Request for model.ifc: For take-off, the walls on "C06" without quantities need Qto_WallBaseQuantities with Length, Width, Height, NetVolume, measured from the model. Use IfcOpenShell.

First a look at what the model holds.

```python
import ifcopenshell
import ifcopenshell.util.element
import ifcopenshell.util.unit

model = ifcopenshell.open("model.ifc")
print(model.schema)
for unit_type in ("LENGTHUNIT", "AREAUNIT", "VOLUMEUNIT"):
    print(unit_type, ifcopenshell.util.unit.calculate_unit_scale(model, unit_type))
storey = next(s for s in model.by_type("IfcBuildingStorey") if s.Name == "C06")
walls = [e for e in ifcopenshell.util.element.get_decomposition(storey) if e.is_a("IfcWall")]
for e in sorted(walls, key=lambda e: e.id()):
    print(e.id(), e.is_a(), e.Name, list(ifcopenshell.util.element.get_psets(e, qtos_only=True)), sep=" | ")
```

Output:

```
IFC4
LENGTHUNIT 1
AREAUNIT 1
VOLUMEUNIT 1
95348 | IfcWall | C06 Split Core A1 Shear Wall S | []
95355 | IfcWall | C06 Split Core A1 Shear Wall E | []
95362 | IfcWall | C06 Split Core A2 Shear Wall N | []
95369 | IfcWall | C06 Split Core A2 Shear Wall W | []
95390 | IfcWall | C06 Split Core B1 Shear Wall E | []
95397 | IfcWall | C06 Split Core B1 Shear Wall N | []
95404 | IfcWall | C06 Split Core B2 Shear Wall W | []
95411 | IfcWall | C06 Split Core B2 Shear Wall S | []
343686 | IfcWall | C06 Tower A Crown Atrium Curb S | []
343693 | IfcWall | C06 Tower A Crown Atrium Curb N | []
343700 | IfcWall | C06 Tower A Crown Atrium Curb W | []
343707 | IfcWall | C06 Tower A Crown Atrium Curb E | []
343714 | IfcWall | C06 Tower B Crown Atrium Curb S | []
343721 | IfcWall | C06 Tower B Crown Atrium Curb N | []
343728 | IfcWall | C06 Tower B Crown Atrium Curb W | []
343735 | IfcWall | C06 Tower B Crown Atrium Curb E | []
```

```python
import ifcopenshell
import ifcopenshell.api.pset
import ifcopenshell.geom
import ifcopenshell.util.element
import ifcopenshell.util.shape
import ifcopenshell.util.unit

model = ifcopenshell.open("model.ifc")
unit_scale = ifcopenshell.util.unit.calculate_unit_scale(model)
volume_scale = ifcopenshell.util.unit.calculate_unit_scale(model, "VOLUMEUNIT")
settings = ifcopenshell.geom.settings()

storey = next(s for s in model.by_type("IfcBuildingStorey") if s.Name == "C06")
walls = [e for e in ifcopenshell.util.element.get_decomposition(storey) if e.is_a("IfcWall")]

for e in sorted(walls, key=lambda e: e.id()):
    if ifcopenshell.util.element.get_psets(e, qtos_only=True, should_inherit=False):
        continue
    # Geometry comes back in metres, in the element's own axes.
    shape = ifcopenshell.geom.create_shape(settings, e)
    values = {
        "Length": ifcopenshell.util.shape.get_x(shape.geometry) / unit_scale,
        "Width": ifcopenshell.util.shape.get_y(shape.geometry) / unit_scale,
        "Height": ifcopenshell.util.shape.get_z(shape.geometry) / unit_scale,
        "NetVolume": ifcopenshell.util.shape.get_volume(shape.geometry) / volume_scale,
    }
    qto = ifcopenshell.api.pset.add_qto(model, product=e, name="Qto_WallBaseQuantities")
    ifcopenshell.api.pset.edit_qto(model, qto=qto, properties=values)
    print(e.id(), {k: round(v, 3) for k, v in values.items()})

model.write("model_updated.ifc")
```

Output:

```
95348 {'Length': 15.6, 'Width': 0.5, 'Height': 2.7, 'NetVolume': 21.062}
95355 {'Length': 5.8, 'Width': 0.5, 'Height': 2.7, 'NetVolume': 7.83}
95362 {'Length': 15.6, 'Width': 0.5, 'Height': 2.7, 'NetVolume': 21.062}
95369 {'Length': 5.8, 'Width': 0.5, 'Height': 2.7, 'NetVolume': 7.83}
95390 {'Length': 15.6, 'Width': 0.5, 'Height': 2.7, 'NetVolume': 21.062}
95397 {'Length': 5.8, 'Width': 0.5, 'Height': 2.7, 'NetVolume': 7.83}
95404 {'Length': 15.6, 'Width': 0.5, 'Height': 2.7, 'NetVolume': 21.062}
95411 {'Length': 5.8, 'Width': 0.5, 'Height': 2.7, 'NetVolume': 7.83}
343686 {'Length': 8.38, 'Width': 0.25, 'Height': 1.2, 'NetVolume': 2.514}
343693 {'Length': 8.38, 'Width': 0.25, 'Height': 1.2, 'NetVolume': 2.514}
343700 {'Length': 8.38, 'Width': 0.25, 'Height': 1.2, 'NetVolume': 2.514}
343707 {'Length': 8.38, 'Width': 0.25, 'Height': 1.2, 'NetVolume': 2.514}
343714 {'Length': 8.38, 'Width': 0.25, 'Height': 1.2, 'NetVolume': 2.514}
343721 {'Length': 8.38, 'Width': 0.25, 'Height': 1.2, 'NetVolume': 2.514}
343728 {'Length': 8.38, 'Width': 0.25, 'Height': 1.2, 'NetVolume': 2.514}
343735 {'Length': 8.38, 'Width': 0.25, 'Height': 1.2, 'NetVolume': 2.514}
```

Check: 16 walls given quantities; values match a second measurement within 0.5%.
